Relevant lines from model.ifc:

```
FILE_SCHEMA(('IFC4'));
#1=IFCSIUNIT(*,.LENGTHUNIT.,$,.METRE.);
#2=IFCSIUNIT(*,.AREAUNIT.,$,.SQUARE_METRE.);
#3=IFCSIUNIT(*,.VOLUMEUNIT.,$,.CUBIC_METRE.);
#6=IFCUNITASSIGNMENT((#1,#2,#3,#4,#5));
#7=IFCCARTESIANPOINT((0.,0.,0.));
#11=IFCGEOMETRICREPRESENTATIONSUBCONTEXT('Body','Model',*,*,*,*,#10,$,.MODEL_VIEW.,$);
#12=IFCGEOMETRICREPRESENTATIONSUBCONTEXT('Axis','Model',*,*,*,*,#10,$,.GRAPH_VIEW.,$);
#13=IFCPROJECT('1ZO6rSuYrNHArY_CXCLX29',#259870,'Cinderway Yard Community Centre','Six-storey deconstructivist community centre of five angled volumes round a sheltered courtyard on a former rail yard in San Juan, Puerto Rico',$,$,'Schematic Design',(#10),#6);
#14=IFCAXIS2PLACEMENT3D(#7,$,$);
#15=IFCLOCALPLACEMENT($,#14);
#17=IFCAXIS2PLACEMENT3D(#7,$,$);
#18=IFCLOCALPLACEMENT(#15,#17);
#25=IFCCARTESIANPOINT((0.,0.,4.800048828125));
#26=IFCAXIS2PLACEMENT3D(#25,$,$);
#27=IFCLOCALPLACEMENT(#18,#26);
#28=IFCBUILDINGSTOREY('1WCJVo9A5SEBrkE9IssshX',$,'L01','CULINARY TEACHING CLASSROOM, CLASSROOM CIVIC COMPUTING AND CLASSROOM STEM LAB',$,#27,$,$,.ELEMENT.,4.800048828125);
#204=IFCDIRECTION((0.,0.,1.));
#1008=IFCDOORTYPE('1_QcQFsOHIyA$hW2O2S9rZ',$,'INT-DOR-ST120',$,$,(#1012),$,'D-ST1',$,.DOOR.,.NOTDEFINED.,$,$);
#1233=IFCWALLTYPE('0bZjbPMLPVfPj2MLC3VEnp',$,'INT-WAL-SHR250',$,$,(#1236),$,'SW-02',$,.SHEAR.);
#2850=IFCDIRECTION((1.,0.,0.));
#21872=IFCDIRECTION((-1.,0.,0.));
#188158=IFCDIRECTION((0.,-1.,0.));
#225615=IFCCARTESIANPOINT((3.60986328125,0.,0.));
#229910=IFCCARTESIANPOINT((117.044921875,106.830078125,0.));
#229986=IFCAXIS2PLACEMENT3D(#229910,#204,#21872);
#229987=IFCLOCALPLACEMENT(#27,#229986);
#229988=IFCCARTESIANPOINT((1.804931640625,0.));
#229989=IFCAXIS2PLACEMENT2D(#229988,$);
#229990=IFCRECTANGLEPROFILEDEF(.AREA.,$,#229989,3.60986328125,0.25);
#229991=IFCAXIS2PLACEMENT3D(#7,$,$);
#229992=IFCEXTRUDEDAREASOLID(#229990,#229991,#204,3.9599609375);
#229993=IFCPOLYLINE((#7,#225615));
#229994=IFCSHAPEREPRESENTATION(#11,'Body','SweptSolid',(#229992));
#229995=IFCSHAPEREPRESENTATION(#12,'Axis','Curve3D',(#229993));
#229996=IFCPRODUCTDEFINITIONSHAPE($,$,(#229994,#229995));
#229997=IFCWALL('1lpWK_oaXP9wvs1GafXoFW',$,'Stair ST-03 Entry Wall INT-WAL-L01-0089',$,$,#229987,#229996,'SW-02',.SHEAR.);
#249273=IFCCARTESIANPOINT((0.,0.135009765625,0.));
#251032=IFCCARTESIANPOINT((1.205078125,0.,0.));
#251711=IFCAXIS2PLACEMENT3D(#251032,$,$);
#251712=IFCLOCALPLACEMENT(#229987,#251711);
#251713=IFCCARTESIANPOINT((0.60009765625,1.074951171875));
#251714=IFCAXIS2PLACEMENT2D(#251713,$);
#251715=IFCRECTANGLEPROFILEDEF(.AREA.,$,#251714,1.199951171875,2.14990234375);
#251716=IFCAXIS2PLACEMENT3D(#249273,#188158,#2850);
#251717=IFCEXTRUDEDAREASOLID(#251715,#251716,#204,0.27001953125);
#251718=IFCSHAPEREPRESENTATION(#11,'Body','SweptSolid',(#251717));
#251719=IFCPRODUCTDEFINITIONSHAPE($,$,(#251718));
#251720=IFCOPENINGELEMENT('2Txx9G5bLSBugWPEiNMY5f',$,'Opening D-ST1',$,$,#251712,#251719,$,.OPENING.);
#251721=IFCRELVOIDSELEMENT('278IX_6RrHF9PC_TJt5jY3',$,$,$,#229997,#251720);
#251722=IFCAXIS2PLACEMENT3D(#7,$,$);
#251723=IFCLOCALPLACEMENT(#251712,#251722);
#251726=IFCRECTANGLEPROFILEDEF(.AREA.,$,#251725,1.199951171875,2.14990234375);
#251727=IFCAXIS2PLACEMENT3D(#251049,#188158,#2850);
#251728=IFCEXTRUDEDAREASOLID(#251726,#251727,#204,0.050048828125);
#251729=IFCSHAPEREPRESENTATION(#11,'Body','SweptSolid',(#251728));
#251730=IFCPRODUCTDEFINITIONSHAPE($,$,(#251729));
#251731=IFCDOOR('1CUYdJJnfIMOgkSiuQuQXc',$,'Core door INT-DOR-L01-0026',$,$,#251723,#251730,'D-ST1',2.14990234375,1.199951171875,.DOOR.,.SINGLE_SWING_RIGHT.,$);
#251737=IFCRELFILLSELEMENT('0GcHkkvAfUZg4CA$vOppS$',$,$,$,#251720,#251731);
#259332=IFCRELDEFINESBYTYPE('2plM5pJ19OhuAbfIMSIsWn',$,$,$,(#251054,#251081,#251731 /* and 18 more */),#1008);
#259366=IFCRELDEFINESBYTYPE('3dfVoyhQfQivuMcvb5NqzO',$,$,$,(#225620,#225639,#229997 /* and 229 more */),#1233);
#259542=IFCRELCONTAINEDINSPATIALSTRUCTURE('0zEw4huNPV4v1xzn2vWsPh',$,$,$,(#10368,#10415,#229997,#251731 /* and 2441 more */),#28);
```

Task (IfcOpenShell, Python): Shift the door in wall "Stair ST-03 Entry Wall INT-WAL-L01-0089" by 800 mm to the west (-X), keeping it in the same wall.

```python
import ifcopenshell
import ifcopenshell.api.geometry
import ifcopenshell.util.placement

model = ifcopenshell.open("model.ifc")

door = model.by_guid("1CUYdJJnfIMOgkSiuQuQXc")
opening = door.FillsVoids[0].RelatingOpeningElement
wall = opening.VoidsElements[0].RelatingBuildingElement

wall_matrix = ifcopenshell.util.placement.get_local_placement(wall.ObjectPlacement)
shift = wall_matrix[:3, 0] * 0.8
before = ifcopenshell.util.placement.get_local_placement(door.ObjectPlacement)[:3, 3].copy()

# The door is placed relative to its opening, so it follows when the opening moves.
matrix = ifcopenshell.util.placement.get_local_placement(opening.ObjectPlacement)
matrix[:3, 3] += shift
ifcopenshell.api.geometry.edit_object_placement(
    model, product=opening, matrix=matrix, is_si=False, should_transform_children=True
)

after = ifcopenshell.util.placement.get_local_placement(door.ObjectPlacement)[:3, 3]
print("door moved by", (after - before).round(3) + 0.0)

model.write("model-out.ifc")
```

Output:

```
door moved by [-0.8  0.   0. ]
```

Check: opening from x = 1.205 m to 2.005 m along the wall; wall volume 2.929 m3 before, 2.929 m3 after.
